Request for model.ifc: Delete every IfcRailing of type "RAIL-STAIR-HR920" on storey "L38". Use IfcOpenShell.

First a look at what the model holds.

```python
import ifcopenshell
import ifcopenshell.util.element

model = ifcopenshell.open("model.ifc")
print(model.schema)
storey = next(s for s in model.by_type("IfcBuildingStorey") if s.Name == "L38")
railings = [e for e in ifcopenshell.util.element.get_decomposition(storey) if e.is_a("IfcRailing")]
seen = {}
for e in railings:
    element_type = ifcopenshell.util.element.get_type(e)
    name = element_type.Name if element_type not in (None, e) else None
    seen[name] = seen.get(name, 0) + 1
for name, count in sorted(seen.items(), key=str):
    print(count, "x", name)
```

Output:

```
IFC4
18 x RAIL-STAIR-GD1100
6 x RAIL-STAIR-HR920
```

```python
import ifcopenshell
import ifcopenshell.api.root
import ifcopenshell.util.element

model = ifcopenshell.open("model.ifc")

storey = next(s for s in model.by_type("IfcBuildingStorey") if s.Name == "L38")
railings = [e for e in ifcopenshell.util.element.get_decomposition(storey) if e.is_a("IfcRailing")]
targets = [e for e in railings if (t := ifcopenshell.util.element.get_type(e)) not in (None, e) and t.Name == "RAIL-STAIR-HR920"]

for e in targets:
    ifcopenshell.api.root.remove_product(model, product=e)
print(len(targets), "removed")

model.write("model_edited.ifc")
```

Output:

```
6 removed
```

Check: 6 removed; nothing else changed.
